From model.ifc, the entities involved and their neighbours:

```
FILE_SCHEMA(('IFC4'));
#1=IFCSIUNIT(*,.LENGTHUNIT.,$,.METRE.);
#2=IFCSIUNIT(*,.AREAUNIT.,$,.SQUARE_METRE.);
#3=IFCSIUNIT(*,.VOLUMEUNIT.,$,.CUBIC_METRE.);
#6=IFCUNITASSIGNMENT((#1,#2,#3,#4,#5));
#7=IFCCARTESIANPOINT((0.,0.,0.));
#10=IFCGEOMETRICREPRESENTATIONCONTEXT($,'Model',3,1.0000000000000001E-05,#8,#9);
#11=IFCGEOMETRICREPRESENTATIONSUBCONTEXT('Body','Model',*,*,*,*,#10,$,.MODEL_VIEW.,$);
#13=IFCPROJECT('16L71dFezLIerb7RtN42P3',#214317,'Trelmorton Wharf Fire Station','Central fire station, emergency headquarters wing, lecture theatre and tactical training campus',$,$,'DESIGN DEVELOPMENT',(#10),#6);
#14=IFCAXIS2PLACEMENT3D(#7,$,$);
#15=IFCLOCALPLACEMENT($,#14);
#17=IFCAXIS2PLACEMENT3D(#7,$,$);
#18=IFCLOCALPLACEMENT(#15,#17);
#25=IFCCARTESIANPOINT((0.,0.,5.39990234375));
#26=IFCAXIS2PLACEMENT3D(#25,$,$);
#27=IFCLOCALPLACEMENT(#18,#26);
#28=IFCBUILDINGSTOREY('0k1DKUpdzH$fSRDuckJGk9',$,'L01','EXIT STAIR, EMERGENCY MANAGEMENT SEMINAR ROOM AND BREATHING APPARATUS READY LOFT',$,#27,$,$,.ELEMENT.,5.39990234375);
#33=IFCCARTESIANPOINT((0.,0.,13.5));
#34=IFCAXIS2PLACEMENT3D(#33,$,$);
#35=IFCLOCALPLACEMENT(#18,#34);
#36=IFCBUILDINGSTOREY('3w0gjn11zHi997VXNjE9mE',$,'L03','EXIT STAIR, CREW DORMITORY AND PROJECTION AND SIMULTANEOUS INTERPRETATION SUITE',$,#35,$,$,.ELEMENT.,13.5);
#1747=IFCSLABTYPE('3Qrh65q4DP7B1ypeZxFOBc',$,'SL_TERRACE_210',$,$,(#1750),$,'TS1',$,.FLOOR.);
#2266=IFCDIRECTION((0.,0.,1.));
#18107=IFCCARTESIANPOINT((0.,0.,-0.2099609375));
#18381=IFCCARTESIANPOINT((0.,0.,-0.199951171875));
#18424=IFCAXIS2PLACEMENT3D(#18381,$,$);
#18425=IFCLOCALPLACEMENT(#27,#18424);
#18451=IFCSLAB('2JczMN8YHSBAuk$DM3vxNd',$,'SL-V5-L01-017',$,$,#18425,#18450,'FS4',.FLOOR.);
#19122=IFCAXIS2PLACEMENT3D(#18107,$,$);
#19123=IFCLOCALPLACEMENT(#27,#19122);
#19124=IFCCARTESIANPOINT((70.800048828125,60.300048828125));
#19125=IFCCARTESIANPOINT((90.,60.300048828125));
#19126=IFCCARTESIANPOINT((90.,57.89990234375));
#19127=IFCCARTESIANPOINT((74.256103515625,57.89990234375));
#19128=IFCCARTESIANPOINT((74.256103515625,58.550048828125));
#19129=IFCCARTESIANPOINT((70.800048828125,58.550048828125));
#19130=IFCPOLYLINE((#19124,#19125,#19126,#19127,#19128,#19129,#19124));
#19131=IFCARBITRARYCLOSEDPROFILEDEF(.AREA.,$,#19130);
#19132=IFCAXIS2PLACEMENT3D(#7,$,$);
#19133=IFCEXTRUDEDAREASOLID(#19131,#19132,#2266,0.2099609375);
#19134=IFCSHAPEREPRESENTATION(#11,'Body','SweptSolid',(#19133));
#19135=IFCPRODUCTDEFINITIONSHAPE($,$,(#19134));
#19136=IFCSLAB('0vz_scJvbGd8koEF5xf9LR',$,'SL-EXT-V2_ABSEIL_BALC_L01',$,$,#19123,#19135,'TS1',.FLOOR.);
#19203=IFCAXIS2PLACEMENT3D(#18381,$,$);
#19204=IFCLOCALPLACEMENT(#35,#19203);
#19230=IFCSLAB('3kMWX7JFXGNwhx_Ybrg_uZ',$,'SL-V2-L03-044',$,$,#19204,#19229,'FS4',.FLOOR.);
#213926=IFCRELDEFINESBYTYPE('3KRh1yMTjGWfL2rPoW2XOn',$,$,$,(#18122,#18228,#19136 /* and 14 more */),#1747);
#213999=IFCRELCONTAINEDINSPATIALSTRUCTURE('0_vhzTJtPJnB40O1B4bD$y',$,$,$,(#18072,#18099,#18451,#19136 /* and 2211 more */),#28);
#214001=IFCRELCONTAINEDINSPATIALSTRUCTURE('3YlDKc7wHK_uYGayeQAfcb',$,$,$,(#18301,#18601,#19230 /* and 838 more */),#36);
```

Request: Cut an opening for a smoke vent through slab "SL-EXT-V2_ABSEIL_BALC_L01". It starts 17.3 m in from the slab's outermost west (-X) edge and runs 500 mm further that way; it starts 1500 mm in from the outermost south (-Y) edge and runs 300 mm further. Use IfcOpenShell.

```python
import numpy as np
import ifcopenshell
import ifcopenshell.api.feature
import ifcopenshell.api.geometry
import ifcopenshell.api.root
import ifcopenshell.geom
import ifcopenshell.util.placement
import ifcopenshell.util.representation
import ifcopenshell.util.shape
import ifcopenshell.util.unit

model = ifcopenshell.open("model.ifc")
unit_scale = ifcopenshell.util.unit.calculate_unit_scale(model)
settings = ifcopenshell.geom.settings()


def volume(element):
    """Net volume in cubic metres, openings subtracted."""
    shape = ifcopenshell.geom.create_shape(settings, element)
    return ifcopenshell.util.shape.get_volume(shape.geometry)


slab = model.by_guid("0vz_scJvbGd8koEF5xf9LR")
before = volume(slab)

# Extent in the slab's own axes, in metres. The edges named are its -X and -Y sides.
slab_shape = ifcopenshell.geom.create_shape(settings, slab)
vertices = ifcopenshell.util.shape.get_vertices(slab_shape.geometry)
x_min, y_min, bottom = vertices.min(axis=0)
top = vertices[:, 2].max()

opening = ifcopenshell.api.root.create_entity(model, ifc_class="IfcOpeningElement", name="Smoke vent opening", predefined_type="OPENING")
context = ifcopenshell.util.representation.get_context(model, "Model", "Body", "MODEL_VIEW")
width, depth = 0.5, 0.3
outline = [(0.0, 0.0), (width, 0.0), (width, depth), (0.0, depth), (0.0, 0.0)]
# Overshoot both faces by 50 mm so the cut is clean.
shape = ifcopenshell.api.geometry.add_slab_representation(
    model, context=context, depth=top - bottom + 0.1, polyline=outline
)
ifcopenshell.api.geometry.assign_representation(model, product=opening, representation=shape)

matrix = ifcopenshell.util.placement.get_local_placement(slab.ObjectPlacement)
matrix[:, 3] = matrix @ np.append(np.array([x_min + 17.3, y_min + 1.5, bottom - 0.05]) / unit_scale, 1.0)
ifcopenshell.api.geometry.edit_object_placement(model, product=opening, matrix=matrix, is_si=False)
ifcopenshell.api.feature.add_feature(model, feature=opening, element=slab)

after = volume(slab)

print(f"slab volume {before:.3f} -> {after:.3f} m3")

model.write("model_v2.ifc")
```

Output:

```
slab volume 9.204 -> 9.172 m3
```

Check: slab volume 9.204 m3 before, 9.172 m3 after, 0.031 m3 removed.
